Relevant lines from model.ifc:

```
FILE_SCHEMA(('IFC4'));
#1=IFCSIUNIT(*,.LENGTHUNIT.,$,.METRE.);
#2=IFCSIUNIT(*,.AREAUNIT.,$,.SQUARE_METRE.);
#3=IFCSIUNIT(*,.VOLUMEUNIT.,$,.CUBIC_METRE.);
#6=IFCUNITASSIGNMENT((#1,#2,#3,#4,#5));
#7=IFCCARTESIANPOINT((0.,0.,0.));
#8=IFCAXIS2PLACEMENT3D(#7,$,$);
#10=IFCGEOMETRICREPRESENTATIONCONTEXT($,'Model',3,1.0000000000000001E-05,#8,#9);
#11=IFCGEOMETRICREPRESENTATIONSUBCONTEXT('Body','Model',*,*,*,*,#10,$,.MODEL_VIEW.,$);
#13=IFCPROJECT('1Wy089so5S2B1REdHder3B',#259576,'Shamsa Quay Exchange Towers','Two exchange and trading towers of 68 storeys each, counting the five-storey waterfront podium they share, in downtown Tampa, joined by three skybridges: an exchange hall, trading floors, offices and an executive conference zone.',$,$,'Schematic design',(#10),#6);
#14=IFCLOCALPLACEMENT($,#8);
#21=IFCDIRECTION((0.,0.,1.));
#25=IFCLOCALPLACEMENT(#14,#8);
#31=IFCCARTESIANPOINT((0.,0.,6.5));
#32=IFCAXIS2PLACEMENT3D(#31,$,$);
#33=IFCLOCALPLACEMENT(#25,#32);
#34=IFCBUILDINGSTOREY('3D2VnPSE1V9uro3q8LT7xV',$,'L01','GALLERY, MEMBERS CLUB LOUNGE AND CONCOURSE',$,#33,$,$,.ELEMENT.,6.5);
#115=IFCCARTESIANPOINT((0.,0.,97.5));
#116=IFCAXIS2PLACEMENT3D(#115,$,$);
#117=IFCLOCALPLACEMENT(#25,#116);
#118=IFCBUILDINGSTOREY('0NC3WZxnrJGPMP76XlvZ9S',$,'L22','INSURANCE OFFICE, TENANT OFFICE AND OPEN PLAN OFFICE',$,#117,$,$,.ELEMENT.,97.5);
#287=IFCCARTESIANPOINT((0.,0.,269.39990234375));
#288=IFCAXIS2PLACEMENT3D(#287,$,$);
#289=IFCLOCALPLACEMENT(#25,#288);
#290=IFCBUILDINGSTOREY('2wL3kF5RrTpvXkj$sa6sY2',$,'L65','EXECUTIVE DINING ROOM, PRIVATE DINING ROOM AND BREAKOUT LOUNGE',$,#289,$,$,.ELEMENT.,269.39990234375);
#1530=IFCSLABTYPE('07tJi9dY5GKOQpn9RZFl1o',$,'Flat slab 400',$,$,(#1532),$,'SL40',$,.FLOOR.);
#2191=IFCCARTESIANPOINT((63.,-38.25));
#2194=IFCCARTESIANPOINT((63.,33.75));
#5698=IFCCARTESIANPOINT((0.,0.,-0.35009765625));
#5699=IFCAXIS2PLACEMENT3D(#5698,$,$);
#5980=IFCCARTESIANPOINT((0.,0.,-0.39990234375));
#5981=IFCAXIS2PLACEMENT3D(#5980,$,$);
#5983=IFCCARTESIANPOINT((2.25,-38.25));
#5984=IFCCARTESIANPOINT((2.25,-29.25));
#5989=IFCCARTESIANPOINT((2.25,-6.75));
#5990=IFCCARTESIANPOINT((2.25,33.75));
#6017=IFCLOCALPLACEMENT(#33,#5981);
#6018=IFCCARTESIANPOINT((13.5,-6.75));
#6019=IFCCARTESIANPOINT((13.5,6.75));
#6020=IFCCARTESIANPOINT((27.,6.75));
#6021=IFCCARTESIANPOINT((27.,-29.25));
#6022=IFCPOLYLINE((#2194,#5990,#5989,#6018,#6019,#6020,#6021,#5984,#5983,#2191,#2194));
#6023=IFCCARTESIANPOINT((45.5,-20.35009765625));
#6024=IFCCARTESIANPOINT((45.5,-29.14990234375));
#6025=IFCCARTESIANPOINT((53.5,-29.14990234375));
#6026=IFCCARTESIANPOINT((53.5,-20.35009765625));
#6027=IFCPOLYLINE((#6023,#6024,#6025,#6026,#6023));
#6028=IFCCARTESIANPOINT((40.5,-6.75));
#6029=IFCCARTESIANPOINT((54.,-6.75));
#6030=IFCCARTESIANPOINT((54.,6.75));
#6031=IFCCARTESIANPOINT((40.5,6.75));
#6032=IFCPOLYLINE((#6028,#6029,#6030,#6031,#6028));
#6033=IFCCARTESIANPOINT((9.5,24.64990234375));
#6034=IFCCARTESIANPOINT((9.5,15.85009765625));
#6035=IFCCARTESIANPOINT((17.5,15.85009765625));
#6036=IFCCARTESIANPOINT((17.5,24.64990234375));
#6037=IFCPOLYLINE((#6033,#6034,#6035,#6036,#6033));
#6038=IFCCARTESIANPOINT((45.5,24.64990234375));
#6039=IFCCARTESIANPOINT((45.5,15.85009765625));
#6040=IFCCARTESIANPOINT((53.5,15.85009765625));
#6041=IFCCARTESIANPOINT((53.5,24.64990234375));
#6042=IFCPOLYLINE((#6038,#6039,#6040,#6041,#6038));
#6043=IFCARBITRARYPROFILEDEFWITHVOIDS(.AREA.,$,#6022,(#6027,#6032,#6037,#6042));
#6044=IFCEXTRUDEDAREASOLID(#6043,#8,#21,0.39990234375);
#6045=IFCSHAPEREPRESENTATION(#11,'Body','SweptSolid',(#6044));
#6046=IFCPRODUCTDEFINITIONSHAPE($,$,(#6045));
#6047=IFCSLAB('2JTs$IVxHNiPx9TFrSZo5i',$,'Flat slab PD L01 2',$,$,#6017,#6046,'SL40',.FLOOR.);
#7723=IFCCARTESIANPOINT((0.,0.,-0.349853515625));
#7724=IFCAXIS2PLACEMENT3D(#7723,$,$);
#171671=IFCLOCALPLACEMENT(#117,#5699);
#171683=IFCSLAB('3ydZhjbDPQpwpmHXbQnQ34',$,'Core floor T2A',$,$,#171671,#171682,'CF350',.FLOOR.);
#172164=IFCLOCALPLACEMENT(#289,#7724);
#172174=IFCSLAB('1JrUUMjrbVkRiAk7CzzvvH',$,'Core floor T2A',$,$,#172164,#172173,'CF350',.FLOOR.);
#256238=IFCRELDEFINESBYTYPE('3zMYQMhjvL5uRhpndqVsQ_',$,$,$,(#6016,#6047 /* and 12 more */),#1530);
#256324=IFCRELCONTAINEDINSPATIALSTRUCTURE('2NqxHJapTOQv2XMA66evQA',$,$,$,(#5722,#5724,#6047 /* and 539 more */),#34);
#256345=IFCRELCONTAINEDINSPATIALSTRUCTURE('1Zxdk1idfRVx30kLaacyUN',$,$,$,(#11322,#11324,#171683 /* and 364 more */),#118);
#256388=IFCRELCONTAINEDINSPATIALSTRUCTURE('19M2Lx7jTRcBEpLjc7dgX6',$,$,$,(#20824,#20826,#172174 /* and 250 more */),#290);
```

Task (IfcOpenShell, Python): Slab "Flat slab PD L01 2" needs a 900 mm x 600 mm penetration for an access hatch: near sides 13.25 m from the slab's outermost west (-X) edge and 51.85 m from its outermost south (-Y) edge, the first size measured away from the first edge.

```python
import numpy as np
import ifcopenshell
import ifcopenshell.api.feature
import ifcopenshell.api.geometry
import ifcopenshell.api.root
import ifcopenshell.geom
import ifcopenshell.util.placement
import ifcopenshell.util.representation
import ifcopenshell.util.shape
import ifcopenshell.util.unit

model = ifcopenshell.open("model.ifc")
unit_scale = ifcopenshell.util.unit.calculate_unit_scale(model)
settings = ifcopenshell.geom.settings()


def volume(element):
    """Net volume in cubic metres, openings subtracted."""
    shape = ifcopenshell.geom.create_shape(settings, element)
    return ifcopenshell.util.shape.get_volume(shape.geometry)


slab = model.by_id(6047)
before = volume(slab)

# Extent in the slab's own axes, in metres. The edges named are its -X and -Y sides.
slab_shape = ifcopenshell.geom.create_shape(settings, slab)
vertices = ifcopenshell.util.shape.get_vertices(slab_shape.geometry)
x_min, y_min, bottom = vertices.min(axis=0)
top = vertices[:, 2].max()

opening = ifcopenshell.api.root.create_entity(model, ifc_class="IfcOpeningElement", name="Access hatch opening", predefined_type="OPENING")
context = ifcopenshell.util.representation.get_context(model, "Model", "Body", "MODEL_VIEW")
width, depth = 0.9, 0.6
outline = [(0.0, 0.0), (width, 0.0), (width, depth), (0.0, depth), (0.0, 0.0)]
# Overshoot both faces by 50 mm so the cut is clean.
shape = ifcopenshell.api.geometry.add_slab_representation(
    model, context=context, depth=top - bottom + 0.1, polyline=outline
)
ifcopenshell.api.geometry.assign_representation(model, product=opening, representation=shape)

matrix = ifcopenshell.util.placement.get_local_placement(slab.ObjectPlacement)
matrix[:, 3] = matrix @ np.append(np.array([x_min + 13.25, y_min + 51.85, bottom - 0.05]) / unit_scale, 1.0)
ifcopenshell.api.geometry.edit_object_placement(model, product=opening, matrix=matrix, is_si=False)
ifcopenshell.api.feature.add_feature(model, feature=opening, element=slab)

after = volume(slab)

print(f"slab volume {before:.3f} -> {after:.3f} m3")

model.write("model_v2.ifc")
```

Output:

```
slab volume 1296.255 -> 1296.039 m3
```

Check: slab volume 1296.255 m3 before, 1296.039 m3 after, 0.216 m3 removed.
